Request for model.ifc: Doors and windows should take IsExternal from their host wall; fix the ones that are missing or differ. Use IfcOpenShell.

First a look at what the model holds.

```python
import ifcopenshell
import ifcopenshell.util.element

model = ifcopenshell.open("model.ifc")
print(model.schema)
seen = {}
for e in model.by_type("IfcDoor") + model.by_type("IfcWindow"):
    if not e.FillsVoids:
        continue
    host = e.FillsVoids[0].RelatingOpeningElement.VoidsElements[0].RelatingBuildingElement
    own = ifcopenshell.util.element.get_pset(e, f"Pset_{e.is_a()[3:].removesuffix('StandardCase')}Common", "IsExternal")
    wall = ifcopenshell.util.element.get_pset(host, "Pset_WallCommon", "IsExternal")
    seen[e.is_a(), own, wall] = seen.get((e.is_a(), own, wall), 0) + 1
for (cls, own, wall), count in sorted(seen.items(), key=str):
    print(count, cls, "IsExternal:", own, "| host wall:", wall)
```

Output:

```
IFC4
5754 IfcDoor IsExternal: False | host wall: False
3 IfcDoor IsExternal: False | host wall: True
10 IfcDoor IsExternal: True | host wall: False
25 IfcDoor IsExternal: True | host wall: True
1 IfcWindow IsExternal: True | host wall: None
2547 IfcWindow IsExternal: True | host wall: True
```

```python
import ifcopenshell
import ifcopenshell.api.pset
import ifcopenshell.util.element

model = ifcopenshell.open("model.ifc")

count = 0
for ifc_class, pset_name in (("IfcDoor", "Pset_DoorCommon"), ("IfcWindow", "Pset_WindowCommon")):
    for e in model.by_type(ifc_class):
        if not e.FillsVoids:
            continue
        host = e.FillsVoids[0].RelatingOpeningElement.VoidsElements[0].RelatingBuildingElement
        external = ifcopenshell.util.element.get_pset(host, "Pset_WallCommon", "IsExternal")
        if external is None or ifcopenshell.util.element.get_pset(e, pset_name, "IsExternal") == external:
            continue
        pset = ifcopenshell.api.pset.add_pset(model, product=e, name=pset_name)
        ifcopenshell.api.pset.edit_pset(model, pset=pset, properties={"IsExternal": external})
        count += 1

print(count, "updated")

model.write("model_rev.ifc")
```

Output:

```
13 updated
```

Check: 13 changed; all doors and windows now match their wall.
